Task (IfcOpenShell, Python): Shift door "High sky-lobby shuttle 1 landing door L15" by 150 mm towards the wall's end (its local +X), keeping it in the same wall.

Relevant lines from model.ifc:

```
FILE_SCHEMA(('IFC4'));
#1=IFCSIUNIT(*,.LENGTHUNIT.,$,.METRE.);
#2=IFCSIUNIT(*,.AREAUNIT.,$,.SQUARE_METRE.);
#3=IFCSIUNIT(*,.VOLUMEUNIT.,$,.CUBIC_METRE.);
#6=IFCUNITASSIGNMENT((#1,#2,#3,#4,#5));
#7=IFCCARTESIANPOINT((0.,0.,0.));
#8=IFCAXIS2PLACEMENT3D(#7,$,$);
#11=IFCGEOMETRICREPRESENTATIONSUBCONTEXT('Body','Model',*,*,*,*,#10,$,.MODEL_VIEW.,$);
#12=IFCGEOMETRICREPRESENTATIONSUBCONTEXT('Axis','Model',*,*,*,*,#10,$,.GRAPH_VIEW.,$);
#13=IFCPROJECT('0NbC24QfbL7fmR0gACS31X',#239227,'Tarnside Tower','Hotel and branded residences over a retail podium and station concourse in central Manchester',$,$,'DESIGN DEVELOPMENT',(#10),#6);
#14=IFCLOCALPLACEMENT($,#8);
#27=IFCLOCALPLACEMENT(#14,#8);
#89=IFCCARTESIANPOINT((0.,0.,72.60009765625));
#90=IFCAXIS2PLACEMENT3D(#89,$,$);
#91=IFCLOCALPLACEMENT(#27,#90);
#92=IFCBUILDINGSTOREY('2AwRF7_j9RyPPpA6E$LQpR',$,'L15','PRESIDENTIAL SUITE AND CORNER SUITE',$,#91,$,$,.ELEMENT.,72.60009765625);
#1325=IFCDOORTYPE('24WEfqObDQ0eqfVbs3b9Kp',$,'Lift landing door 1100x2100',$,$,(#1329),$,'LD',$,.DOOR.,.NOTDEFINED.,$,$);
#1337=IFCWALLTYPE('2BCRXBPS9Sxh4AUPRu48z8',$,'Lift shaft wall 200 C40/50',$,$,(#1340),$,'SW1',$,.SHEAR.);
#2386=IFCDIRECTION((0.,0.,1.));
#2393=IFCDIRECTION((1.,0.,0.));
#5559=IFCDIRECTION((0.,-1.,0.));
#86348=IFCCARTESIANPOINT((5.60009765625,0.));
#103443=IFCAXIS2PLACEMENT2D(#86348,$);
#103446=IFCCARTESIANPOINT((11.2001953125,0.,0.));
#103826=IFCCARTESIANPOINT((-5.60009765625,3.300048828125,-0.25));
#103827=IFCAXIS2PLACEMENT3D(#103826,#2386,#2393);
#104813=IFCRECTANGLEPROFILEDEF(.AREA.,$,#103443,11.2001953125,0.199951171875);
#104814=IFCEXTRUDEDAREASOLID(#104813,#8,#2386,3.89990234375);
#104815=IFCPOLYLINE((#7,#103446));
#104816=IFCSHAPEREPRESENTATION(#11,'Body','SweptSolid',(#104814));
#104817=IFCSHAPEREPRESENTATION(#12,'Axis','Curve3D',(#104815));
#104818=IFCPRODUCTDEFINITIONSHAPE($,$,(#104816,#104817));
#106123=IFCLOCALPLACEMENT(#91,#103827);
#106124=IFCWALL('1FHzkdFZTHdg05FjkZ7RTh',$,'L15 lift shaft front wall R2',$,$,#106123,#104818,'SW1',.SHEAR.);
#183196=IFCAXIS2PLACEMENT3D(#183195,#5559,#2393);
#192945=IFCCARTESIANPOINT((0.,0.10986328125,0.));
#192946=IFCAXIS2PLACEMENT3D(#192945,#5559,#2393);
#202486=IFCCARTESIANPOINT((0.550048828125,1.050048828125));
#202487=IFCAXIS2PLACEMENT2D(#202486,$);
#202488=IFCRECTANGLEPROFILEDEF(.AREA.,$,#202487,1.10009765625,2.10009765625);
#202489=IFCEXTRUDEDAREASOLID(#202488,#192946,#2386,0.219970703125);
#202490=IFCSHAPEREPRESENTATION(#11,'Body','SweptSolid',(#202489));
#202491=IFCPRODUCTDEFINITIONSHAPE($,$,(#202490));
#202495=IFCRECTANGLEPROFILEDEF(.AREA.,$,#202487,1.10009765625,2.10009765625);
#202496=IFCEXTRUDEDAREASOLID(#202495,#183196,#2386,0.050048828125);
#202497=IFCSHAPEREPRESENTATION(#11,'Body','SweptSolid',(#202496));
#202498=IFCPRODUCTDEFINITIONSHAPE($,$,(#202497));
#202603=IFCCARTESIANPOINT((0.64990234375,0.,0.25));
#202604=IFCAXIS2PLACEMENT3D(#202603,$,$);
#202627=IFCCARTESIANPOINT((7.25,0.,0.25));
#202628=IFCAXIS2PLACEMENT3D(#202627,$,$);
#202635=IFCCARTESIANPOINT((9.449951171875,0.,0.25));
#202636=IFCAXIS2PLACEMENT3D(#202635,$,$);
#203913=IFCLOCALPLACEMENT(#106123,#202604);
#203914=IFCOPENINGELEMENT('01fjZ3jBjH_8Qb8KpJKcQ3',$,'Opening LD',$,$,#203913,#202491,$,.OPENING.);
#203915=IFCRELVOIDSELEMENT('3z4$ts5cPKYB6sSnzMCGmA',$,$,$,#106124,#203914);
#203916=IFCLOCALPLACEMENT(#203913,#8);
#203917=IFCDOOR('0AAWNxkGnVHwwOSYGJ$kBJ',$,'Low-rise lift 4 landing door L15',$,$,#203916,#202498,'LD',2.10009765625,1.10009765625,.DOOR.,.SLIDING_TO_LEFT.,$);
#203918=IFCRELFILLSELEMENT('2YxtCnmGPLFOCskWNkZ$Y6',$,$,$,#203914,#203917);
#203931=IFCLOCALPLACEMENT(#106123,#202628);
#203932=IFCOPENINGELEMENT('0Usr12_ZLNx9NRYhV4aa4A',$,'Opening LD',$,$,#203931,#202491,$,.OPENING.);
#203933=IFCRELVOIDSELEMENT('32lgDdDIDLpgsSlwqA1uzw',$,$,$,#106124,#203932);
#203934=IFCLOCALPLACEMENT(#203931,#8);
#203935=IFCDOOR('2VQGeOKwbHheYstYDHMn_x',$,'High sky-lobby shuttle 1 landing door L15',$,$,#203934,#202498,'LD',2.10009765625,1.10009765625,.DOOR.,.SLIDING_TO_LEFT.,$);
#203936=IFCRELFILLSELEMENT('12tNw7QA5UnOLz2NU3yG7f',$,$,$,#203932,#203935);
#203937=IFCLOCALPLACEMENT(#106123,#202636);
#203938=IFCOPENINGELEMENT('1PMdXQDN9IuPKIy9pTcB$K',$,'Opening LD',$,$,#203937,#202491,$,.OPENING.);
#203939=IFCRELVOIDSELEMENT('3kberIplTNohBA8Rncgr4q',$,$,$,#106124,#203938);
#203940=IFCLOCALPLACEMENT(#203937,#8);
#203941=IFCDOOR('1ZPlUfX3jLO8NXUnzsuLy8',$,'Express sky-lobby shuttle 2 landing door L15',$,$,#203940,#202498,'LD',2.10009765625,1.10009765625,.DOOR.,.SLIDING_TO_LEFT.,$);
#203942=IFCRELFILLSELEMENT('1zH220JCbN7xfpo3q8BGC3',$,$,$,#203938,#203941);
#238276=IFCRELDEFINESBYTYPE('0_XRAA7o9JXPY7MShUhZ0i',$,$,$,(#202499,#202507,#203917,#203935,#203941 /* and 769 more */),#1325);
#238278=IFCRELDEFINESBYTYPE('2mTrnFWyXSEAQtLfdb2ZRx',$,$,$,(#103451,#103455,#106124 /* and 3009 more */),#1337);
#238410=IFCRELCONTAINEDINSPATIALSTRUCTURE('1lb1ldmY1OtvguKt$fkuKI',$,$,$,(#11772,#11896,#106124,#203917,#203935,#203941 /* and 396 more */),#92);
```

```python
import ifcopenshell
import ifcopenshell.api.geometry
import ifcopenshell.util.placement
import ifcopenshell.util.unit

model = ifcopenshell.open("model.ifc")
unit_scale = ifcopenshell.util.unit.calculate_unit_scale(model)

door = model.by_guid("2VQGeOKwbHheYstYDHMn_x")
opening = door.FillsVoids[0].RelatingOpeningElement
wall = opening.VoidsElements[0].RelatingBuildingElement

wall_matrix = ifcopenshell.util.placement.get_local_placement(wall.ObjectPlacement)
shift = wall_matrix[:3, 0] * 0.15 / unit_scale
before = ifcopenshell.util.placement.get_local_placement(door.ObjectPlacement)[:3, 3].copy()

# The door is placed relative to its opening, so it follows when the opening moves.
matrix = ifcopenshell.util.placement.get_local_placement(opening.ObjectPlacement)
matrix[:3, 3] += shift
ifcopenshell.api.geometry.edit_object_placement(
    model, product=opening, matrix=matrix, is_si=False, should_transform_children=True
)

after = ifcopenshell.util.placement.get_local_placement(door.ObjectPlacement)[:3, 3]
print("door moved by", (after - before).round(3) + 0.0)

model.write("model_rev.ifc")
```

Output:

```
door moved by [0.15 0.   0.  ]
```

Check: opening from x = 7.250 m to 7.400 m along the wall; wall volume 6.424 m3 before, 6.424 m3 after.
